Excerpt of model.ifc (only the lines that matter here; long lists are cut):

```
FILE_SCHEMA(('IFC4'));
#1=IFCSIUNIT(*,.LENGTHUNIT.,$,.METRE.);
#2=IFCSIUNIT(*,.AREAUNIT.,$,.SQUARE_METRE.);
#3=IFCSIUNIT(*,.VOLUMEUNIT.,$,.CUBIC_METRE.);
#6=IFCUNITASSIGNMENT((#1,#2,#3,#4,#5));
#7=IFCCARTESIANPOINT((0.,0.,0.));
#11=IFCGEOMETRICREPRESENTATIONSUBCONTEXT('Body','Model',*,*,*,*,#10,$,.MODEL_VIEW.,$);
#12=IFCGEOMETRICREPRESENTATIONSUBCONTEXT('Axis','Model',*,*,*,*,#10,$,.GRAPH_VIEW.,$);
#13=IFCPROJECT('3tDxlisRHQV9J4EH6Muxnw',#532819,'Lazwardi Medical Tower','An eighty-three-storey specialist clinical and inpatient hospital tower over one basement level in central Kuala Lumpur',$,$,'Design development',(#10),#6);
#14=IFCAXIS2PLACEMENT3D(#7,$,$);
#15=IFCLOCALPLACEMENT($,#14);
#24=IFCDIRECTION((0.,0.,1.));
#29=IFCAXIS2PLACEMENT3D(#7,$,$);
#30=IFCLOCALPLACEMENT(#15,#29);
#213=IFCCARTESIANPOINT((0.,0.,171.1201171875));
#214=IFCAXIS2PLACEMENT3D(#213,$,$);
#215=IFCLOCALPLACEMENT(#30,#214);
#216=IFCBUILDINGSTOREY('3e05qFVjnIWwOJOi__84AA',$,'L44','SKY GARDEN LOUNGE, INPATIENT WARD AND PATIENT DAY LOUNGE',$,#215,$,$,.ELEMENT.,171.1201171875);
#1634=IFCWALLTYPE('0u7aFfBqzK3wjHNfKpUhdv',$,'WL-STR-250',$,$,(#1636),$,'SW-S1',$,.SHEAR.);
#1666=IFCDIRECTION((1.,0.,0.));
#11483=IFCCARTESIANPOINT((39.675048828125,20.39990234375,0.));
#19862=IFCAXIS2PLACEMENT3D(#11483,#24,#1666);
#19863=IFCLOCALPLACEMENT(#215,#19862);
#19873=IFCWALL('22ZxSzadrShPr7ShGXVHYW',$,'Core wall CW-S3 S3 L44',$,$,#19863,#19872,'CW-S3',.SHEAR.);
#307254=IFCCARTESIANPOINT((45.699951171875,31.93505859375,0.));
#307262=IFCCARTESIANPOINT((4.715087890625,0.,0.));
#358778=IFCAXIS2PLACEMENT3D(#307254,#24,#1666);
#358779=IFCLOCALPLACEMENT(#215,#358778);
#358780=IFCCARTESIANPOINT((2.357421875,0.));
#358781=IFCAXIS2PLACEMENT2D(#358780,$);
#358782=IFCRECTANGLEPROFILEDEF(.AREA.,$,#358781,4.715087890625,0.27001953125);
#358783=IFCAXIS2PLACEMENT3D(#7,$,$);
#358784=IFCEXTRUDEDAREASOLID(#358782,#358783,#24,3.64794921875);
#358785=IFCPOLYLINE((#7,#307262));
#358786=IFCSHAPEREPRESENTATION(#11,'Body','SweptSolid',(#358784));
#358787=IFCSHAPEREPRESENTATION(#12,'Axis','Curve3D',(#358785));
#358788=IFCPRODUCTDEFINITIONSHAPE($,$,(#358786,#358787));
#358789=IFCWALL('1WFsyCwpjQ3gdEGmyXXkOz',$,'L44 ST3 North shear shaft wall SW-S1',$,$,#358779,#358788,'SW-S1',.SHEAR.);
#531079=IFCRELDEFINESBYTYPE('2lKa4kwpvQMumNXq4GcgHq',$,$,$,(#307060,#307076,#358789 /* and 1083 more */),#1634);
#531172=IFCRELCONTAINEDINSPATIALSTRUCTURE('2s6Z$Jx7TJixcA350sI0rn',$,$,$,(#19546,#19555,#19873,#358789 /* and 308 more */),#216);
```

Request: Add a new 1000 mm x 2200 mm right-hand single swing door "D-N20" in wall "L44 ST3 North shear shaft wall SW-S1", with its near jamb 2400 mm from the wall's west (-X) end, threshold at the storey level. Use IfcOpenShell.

```python
import numpy as np
import ifcopenshell
import ifcopenshell.api.feature
import ifcopenshell.api.geometry
import ifcopenshell.api.root
import ifcopenshell.api.spatial
import ifcopenshell.geom
import ifcopenshell.util.element
import ifcopenshell.util.placement
import ifcopenshell.util.representation
import ifcopenshell.util.shape
import ifcopenshell.util.unit

model = ifcopenshell.open("model.ifc")
unit_scale = ifcopenshell.util.unit.calculate_unit_scale(model)
settings = ifcopenshell.geom.settings()


def volume(element):
    """Net volume in cubic metres, openings subtracted."""
    shape = ifcopenshell.geom.create_shape(settings, element)
    return ifcopenshell.util.shape.get_volume(shape.geometry)


wall = model.by_guid("1WFsyCwpjQ3gdEGmyXXkOz")
storey = ifcopenshell.util.element.get_container(wall, ifc_class="IfcBuildingStorey")
context = ifcopenshell.util.representation.get_context(model, "Model", "Body", "MODEL_VIEW")
before = volume(wall)

width, height, from_end, sill = 1, 2.2, 2.4, 0.0  # metres

# The wall runs along its own X axis, and the end named is its -X end.
wall_shape = ifcopenshell.geom.create_shape(settings, wall)
x, y, z = ifcopenshell.util.shape.get_vertices(wall_shape.geometry).T
start = x.min() + from_end
face, thickness = float(y.min()), float(y.max() - y.min())
wall_matrix = ifcopenshell.util.placement.get_local_placement(wall.ObjectPlacement)
level = ifcopenshell.util.placement.get_local_placement(storey.ObjectPlacement)[2, 3]


def in_wall(x, y):
    """Placement at x, y metres in the wall's axes, at sill height."""
    matrix = wall_matrix.copy()
    matrix[:, 3] = wall_matrix @ np.array([x / unit_scale, y / unit_scale, 0.0, 1.0])
    matrix[2, 3] = level + sill / unit_scale
    return matrix


# Opening: a box that overshoots both wall faces by 50 mm.
opening = ifcopenshell.api.root.create_entity(model, ifc_class="IfcOpeningElement", predefined_type="OPENING")
box = ifcopenshell.api.geometry.add_wall_representation(
    model, context=context, length=width, height=height, thickness=thickness + 0.1
)
ifcopenshell.api.geometry.assign_representation(model, product=opening, representation=box)
ifcopenshell.api.geometry.edit_object_placement(model, product=opening, matrix=in_wall(start, face - 0.05), is_si=False)
ifcopenshell.api.feature.add_feature(model, feature=opening, element=wall)

door = ifcopenshell.api.root.create_entity(model, ifc_class="IfcDoor", name="D-N20", predefined_type="DOOR")
door.OverallWidth, door.OverallHeight = width / unit_scale, height / unit_scale
door.OperationType = "SINGLE_SWING_RIGHT"
body = ifcopenshell.api.geometry.add_door_representation(
    model,
    context=context,
    overall_width=door.OverallWidth,
    overall_height=door.OverallHeight,
    operation_type="SINGLE_SWING_RIGHT",
    lining_properties={"LiningDepth": thickness / unit_scale, "ThresholdDepth": thickness / unit_scale},
)
ifcopenshell.api.geometry.assign_representation(model, product=door, representation=body)
ifcopenshell.api.spatial.assign_container(model, products=[door], relating_structure=storey)
ifcopenshell.api.feature.add_filling(model, opening=opening, element=door)

# The lining spans the wall, so the door starts at the wall face.
ifcopenshell.api.geometry.edit_object_placement(model, product=door, matrix=in_wall(start, face), is_si=False)

after = volume(wall)

print(f"wall volume {before:.3f} -> {after:.3f} m3")

model.write("model_v2.ifc")
```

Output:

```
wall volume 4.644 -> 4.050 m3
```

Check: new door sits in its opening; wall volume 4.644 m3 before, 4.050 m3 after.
